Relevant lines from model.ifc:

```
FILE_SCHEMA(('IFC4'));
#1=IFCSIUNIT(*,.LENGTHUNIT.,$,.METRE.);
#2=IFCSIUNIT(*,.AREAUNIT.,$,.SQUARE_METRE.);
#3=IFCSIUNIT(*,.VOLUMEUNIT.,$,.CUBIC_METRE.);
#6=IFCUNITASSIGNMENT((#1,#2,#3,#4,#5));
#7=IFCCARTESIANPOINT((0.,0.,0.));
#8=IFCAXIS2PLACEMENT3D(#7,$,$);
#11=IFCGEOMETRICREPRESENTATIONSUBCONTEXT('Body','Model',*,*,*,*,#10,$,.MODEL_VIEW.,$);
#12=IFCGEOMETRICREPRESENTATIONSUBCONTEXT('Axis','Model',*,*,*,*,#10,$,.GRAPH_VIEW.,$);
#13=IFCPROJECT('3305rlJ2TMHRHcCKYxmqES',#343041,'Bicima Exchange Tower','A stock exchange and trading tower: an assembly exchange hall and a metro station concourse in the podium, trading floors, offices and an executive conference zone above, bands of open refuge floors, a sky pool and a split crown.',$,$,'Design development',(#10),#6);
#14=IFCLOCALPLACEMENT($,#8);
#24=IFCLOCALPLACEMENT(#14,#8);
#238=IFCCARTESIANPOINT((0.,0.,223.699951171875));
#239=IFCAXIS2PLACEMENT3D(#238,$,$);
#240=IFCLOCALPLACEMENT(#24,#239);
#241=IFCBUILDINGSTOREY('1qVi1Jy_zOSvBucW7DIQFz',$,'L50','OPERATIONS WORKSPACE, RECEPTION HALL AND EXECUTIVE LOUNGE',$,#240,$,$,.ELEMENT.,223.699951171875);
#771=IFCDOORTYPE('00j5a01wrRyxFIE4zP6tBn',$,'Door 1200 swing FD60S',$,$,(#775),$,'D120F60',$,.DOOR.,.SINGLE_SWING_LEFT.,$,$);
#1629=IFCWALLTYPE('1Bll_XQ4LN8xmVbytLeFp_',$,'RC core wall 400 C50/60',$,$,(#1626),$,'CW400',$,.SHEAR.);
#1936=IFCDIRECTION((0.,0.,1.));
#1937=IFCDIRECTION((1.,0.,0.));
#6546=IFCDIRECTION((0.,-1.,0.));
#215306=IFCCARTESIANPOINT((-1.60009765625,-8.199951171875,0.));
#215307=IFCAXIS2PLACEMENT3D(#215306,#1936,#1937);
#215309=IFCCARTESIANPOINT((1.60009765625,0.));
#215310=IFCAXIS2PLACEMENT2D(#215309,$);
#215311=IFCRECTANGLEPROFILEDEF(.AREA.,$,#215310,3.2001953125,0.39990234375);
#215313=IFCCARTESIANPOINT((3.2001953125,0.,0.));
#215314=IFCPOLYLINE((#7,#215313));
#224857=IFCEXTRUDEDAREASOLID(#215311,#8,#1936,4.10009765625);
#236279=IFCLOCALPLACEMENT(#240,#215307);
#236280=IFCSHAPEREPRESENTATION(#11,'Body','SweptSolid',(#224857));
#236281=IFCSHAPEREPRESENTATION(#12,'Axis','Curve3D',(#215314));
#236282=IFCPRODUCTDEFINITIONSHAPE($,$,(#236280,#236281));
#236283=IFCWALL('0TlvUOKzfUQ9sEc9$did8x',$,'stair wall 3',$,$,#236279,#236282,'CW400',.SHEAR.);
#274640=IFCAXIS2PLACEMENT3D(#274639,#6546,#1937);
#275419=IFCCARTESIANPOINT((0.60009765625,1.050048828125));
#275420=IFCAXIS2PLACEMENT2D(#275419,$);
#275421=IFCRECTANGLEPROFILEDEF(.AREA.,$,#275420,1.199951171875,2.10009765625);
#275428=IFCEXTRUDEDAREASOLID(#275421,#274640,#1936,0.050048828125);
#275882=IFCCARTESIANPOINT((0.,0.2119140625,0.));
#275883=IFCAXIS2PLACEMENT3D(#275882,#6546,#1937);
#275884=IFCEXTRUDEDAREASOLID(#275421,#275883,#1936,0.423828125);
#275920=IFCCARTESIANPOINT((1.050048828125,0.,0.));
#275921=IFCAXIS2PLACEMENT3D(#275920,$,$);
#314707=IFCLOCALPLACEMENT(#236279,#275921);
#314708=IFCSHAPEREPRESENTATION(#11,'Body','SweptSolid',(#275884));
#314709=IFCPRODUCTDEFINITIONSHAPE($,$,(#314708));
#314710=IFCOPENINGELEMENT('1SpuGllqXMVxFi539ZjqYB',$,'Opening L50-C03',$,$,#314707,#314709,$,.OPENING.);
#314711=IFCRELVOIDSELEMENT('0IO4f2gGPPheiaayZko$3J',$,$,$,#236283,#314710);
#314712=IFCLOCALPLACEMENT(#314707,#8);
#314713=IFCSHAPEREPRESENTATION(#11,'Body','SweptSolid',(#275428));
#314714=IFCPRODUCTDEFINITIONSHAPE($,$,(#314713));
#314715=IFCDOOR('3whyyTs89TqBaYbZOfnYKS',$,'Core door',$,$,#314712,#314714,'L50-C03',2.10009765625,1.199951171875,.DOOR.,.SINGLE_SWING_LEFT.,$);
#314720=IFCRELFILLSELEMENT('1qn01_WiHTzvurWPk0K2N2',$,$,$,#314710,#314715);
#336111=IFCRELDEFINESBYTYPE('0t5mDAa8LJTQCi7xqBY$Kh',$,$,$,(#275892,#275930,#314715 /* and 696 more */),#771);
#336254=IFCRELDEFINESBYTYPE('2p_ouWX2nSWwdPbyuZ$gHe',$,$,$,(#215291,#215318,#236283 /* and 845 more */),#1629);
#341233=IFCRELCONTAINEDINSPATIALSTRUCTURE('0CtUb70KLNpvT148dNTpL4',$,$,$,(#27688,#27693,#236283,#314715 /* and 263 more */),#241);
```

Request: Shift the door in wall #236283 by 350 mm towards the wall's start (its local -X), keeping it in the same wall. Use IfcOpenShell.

```python
import ifcopenshell
import ifcopenshell.api.geometry
import ifcopenshell.util.placement
import ifcopenshell.util.unit

model = ifcopenshell.open("model.ifc")
unit_scale = ifcopenshell.util.unit.calculate_unit_scale(model)

door = model.by_guid("3whyyTs89TqBaYbZOfnYKS")
opening = door.FillsVoids[0].RelatingOpeningElement
wall = opening.VoidsElements[0].RelatingBuildingElement

wall_matrix = ifcopenshell.util.placement.get_local_placement(wall.ObjectPlacement)
shift = wall_matrix[:3, 0] * -0.35 / unit_scale
before = ifcopenshell.util.placement.get_local_placement(door.ObjectPlacement)[:3, 3].copy()

# The door is placed relative to its opening, so it follows when the opening moves.
matrix = ifcopenshell.util.placement.get_local_placement(opening.ObjectPlacement)
matrix[:3, 3] += shift
ifcopenshell.api.geometry.edit_object_placement(
    model, product=opening, matrix=matrix, is_si=False, should_transform_children=True
)

after = ifcopenshell.util.placement.get_local_placement(door.ObjectPlacement)[:3, 3]
print("door moved by", (after - before).round(3) + 0.0)

model.write("model-out.ifc")
```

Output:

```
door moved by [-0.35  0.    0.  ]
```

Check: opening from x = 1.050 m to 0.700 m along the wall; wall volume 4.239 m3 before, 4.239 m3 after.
